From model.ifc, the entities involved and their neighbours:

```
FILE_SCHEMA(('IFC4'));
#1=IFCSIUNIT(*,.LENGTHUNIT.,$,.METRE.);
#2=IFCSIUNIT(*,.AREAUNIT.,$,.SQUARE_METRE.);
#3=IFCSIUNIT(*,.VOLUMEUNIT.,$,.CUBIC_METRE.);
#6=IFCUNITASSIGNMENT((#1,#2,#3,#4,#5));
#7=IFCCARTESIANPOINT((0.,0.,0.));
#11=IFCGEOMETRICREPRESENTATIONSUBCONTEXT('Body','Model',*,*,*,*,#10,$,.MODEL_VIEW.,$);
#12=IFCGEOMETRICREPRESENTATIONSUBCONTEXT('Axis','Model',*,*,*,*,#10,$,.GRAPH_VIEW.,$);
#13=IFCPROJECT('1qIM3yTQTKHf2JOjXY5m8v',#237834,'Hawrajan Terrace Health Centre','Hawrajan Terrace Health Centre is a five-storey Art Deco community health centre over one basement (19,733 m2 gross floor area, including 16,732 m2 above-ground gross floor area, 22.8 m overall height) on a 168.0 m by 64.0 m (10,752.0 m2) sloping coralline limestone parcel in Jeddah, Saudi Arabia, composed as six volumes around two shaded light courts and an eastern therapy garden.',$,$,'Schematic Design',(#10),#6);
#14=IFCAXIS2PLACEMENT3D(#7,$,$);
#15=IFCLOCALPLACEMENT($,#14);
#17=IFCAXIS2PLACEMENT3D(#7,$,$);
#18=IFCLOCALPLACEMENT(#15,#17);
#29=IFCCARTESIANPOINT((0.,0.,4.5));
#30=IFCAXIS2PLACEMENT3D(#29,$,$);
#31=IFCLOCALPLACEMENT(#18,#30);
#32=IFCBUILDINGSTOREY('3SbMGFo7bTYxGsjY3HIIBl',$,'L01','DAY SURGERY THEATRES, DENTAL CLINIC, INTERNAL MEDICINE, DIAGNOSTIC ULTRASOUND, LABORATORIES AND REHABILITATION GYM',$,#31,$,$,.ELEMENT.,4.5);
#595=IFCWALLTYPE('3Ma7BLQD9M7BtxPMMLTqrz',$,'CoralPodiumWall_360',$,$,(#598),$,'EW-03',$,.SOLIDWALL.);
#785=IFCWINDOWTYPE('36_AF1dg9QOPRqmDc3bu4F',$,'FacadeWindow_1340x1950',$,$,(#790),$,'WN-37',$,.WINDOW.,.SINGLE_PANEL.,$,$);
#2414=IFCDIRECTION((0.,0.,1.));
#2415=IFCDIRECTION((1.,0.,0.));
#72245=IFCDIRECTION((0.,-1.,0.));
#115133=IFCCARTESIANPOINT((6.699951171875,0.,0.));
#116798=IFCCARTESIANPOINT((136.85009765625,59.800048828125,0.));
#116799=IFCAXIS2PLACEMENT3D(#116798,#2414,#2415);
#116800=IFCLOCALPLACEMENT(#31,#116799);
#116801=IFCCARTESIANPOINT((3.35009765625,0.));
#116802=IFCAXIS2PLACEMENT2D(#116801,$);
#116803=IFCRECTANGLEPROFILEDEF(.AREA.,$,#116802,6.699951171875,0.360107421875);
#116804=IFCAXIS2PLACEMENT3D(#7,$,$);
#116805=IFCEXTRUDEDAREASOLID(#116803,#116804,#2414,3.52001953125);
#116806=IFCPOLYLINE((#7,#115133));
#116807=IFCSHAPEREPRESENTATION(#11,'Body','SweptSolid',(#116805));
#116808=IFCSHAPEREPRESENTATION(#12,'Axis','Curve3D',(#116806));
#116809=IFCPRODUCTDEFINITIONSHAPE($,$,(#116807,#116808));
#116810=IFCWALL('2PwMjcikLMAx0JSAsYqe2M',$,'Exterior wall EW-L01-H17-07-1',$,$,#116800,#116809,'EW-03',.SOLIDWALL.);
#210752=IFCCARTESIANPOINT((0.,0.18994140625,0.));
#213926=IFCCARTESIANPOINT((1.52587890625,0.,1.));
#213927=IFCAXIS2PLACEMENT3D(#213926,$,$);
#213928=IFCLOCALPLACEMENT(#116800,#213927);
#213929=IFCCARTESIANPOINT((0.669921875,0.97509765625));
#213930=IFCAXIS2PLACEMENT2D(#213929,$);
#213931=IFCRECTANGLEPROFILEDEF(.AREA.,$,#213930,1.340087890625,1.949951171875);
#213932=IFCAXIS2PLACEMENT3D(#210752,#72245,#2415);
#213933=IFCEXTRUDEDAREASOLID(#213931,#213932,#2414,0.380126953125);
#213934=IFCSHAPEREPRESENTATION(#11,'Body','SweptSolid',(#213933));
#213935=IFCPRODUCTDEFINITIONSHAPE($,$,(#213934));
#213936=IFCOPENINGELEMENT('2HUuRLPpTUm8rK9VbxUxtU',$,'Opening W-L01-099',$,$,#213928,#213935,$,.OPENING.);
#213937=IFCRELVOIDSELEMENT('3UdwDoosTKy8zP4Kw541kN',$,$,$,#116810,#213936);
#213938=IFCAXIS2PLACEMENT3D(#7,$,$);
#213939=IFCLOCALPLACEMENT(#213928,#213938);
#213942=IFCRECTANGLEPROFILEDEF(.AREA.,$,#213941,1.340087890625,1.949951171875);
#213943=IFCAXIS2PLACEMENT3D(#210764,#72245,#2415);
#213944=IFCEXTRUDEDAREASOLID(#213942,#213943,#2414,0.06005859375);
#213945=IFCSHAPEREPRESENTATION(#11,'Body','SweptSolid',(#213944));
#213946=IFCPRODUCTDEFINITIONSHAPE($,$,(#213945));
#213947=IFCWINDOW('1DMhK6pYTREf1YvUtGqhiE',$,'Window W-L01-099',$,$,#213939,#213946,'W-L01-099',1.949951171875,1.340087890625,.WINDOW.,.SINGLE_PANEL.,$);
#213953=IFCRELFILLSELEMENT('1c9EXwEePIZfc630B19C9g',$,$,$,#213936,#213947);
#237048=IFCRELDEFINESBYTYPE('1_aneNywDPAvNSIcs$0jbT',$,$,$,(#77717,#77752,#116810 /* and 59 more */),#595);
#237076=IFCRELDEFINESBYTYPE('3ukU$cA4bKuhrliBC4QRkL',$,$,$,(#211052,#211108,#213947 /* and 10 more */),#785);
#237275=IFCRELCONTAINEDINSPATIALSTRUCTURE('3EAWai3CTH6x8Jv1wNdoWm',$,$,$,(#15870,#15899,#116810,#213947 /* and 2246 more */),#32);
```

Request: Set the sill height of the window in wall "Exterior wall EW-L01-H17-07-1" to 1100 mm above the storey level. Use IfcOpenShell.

```python
import numpy as np
import ifcopenshell
import ifcopenshell.api.geometry
import ifcopenshell.geom
import ifcopenshell.util.element
import ifcopenshell.util.placement
import ifcopenshell.util.shape
import ifcopenshell.util.unit

model = ifcopenshell.open("model.ifc")
unit_scale = ifcopenshell.util.unit.calculate_unit_scale(model)

window = model.by_id(213947)
opening = window.FillsVoids[0].RelatingOpeningElement
storey = ifcopenshell.util.element.get_container(window, ifc_class="IfcBuildingStorey")
level = ifcopenshell.util.placement.get_local_placement(storey.ObjectPlacement)[2, 3]

# The opening's origin need not be at the sill, so measure its lowest point.
shape = ifcopenshell.geom.create_shape(ifcopenshell.geom.settings(), opening)
bottom = ifcopenshell.util.shape.get_shape_bottom_elevation(shape, shape.geometry) / unit_scale
dz = level + 1.1 - bottom

shift = np.array([0.0, 0.0, dz])
# The window is placed relative to its opening, so it follows when the opening moves.
matrix = ifcopenshell.util.placement.get_local_placement(opening.ObjectPlacement)
matrix[:3, 3] += shift
ifcopenshell.api.geometry.edit_object_placement(
    model, product=opening, matrix=matrix, is_si=False, should_transform_children=True
)

print(f"moved by {dz * unit_scale:+.3f} m")

model.write("model_rev.ifc")
```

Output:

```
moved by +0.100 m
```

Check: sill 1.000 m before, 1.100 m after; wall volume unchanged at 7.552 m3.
